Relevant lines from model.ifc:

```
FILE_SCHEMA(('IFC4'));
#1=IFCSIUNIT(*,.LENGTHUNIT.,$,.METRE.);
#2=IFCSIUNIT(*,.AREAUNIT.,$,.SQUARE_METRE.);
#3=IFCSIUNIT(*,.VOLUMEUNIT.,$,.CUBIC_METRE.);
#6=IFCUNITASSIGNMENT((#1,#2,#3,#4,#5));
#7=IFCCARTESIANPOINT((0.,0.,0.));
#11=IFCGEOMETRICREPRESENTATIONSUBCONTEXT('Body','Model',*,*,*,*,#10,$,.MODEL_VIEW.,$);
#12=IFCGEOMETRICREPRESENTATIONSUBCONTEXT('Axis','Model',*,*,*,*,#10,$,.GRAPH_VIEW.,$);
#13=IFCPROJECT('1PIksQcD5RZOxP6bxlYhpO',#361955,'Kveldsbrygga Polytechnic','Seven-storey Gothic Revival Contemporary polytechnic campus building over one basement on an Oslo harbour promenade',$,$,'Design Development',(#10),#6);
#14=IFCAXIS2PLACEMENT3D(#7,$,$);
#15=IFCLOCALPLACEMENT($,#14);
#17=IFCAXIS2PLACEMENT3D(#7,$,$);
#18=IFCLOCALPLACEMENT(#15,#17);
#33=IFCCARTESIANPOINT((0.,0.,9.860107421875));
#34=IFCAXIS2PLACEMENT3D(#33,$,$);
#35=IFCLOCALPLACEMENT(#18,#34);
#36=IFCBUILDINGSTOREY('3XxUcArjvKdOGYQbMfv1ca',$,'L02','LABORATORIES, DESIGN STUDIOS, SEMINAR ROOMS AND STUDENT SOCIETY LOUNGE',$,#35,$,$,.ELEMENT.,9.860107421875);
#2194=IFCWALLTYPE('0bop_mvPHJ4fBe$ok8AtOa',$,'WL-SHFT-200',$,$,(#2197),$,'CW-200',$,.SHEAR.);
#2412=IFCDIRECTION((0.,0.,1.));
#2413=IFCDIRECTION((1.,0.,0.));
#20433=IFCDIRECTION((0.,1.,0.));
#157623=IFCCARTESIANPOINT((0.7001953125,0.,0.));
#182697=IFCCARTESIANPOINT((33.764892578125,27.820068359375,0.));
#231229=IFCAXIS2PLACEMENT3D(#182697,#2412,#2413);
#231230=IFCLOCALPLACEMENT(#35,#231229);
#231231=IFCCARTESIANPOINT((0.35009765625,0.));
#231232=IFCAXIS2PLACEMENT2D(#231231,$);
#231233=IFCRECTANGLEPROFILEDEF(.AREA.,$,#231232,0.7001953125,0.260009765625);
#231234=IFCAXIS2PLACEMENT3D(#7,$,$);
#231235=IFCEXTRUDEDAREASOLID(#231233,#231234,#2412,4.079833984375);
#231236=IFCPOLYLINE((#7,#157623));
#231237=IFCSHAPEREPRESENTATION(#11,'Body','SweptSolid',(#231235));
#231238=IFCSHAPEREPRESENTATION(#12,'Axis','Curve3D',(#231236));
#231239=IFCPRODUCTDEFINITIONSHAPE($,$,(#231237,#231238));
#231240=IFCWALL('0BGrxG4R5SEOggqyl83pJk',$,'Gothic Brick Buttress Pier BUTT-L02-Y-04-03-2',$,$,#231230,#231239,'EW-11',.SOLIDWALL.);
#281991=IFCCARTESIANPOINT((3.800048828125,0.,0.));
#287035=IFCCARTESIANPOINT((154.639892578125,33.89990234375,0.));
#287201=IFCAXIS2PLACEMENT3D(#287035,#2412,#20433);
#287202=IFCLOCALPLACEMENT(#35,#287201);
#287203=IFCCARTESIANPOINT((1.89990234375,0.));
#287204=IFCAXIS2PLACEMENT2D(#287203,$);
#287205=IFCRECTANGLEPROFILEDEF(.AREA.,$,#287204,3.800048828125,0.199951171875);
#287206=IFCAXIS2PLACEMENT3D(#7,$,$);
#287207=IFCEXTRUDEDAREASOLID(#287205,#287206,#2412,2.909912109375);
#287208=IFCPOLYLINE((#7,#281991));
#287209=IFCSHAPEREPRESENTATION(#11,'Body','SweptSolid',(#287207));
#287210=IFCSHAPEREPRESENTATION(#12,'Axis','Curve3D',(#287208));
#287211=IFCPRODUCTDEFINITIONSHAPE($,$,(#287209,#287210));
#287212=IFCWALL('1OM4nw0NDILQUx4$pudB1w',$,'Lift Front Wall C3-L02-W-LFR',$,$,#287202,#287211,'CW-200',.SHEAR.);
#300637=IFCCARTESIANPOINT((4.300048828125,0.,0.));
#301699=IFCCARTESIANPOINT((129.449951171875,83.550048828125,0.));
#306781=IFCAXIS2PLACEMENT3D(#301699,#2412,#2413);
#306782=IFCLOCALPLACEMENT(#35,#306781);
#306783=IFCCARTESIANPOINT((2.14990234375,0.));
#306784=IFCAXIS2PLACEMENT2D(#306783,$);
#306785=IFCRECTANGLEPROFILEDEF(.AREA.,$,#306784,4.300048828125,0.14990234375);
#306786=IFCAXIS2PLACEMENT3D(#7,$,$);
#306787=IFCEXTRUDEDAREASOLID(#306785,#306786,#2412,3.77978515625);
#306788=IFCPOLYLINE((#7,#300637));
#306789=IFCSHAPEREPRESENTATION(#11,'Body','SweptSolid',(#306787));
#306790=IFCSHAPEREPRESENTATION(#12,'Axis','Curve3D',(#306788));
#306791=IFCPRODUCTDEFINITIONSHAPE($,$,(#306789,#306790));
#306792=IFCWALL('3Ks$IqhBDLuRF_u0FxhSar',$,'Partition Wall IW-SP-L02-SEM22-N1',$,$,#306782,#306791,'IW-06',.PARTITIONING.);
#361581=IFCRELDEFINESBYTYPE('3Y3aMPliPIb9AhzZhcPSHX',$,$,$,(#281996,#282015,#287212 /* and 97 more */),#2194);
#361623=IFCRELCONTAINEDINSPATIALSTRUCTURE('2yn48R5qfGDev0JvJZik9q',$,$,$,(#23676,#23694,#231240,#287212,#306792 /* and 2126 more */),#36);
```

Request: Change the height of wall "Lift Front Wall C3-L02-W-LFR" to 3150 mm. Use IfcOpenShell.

```python
import ifcopenshell
import ifcopenshell.geom
import ifcopenshell.util.representation
import ifcopenshell.util.shape

model = ifcopenshell.open("model.ifc")
settings = ifcopenshell.geom.settings()


def volume(element):
    """Net volume in cubic metres, openings subtracted."""
    shape = ifcopenshell.geom.create_shape(settings, element)
    return ifcopenshell.util.shape.get_volume(shape.geometry)


wall = model.by_guid("1OM4nw0NDILQUx4$pudB1w")
before = volume(wall)

body = ifcopenshell.util.representation.get_representation(wall, "Model", "Body")
solid = body.Items[0]
old_height = solid.Depth
solid.Depth = 3.15
after = volume(wall)

print(f"height {old_height:g} -> {solid.Depth:g}, volume {before:.3f} -> {after:.3f} m3")

model.write("model_v2.ifc")
```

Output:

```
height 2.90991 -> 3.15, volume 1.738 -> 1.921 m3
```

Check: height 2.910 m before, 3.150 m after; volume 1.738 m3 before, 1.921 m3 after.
